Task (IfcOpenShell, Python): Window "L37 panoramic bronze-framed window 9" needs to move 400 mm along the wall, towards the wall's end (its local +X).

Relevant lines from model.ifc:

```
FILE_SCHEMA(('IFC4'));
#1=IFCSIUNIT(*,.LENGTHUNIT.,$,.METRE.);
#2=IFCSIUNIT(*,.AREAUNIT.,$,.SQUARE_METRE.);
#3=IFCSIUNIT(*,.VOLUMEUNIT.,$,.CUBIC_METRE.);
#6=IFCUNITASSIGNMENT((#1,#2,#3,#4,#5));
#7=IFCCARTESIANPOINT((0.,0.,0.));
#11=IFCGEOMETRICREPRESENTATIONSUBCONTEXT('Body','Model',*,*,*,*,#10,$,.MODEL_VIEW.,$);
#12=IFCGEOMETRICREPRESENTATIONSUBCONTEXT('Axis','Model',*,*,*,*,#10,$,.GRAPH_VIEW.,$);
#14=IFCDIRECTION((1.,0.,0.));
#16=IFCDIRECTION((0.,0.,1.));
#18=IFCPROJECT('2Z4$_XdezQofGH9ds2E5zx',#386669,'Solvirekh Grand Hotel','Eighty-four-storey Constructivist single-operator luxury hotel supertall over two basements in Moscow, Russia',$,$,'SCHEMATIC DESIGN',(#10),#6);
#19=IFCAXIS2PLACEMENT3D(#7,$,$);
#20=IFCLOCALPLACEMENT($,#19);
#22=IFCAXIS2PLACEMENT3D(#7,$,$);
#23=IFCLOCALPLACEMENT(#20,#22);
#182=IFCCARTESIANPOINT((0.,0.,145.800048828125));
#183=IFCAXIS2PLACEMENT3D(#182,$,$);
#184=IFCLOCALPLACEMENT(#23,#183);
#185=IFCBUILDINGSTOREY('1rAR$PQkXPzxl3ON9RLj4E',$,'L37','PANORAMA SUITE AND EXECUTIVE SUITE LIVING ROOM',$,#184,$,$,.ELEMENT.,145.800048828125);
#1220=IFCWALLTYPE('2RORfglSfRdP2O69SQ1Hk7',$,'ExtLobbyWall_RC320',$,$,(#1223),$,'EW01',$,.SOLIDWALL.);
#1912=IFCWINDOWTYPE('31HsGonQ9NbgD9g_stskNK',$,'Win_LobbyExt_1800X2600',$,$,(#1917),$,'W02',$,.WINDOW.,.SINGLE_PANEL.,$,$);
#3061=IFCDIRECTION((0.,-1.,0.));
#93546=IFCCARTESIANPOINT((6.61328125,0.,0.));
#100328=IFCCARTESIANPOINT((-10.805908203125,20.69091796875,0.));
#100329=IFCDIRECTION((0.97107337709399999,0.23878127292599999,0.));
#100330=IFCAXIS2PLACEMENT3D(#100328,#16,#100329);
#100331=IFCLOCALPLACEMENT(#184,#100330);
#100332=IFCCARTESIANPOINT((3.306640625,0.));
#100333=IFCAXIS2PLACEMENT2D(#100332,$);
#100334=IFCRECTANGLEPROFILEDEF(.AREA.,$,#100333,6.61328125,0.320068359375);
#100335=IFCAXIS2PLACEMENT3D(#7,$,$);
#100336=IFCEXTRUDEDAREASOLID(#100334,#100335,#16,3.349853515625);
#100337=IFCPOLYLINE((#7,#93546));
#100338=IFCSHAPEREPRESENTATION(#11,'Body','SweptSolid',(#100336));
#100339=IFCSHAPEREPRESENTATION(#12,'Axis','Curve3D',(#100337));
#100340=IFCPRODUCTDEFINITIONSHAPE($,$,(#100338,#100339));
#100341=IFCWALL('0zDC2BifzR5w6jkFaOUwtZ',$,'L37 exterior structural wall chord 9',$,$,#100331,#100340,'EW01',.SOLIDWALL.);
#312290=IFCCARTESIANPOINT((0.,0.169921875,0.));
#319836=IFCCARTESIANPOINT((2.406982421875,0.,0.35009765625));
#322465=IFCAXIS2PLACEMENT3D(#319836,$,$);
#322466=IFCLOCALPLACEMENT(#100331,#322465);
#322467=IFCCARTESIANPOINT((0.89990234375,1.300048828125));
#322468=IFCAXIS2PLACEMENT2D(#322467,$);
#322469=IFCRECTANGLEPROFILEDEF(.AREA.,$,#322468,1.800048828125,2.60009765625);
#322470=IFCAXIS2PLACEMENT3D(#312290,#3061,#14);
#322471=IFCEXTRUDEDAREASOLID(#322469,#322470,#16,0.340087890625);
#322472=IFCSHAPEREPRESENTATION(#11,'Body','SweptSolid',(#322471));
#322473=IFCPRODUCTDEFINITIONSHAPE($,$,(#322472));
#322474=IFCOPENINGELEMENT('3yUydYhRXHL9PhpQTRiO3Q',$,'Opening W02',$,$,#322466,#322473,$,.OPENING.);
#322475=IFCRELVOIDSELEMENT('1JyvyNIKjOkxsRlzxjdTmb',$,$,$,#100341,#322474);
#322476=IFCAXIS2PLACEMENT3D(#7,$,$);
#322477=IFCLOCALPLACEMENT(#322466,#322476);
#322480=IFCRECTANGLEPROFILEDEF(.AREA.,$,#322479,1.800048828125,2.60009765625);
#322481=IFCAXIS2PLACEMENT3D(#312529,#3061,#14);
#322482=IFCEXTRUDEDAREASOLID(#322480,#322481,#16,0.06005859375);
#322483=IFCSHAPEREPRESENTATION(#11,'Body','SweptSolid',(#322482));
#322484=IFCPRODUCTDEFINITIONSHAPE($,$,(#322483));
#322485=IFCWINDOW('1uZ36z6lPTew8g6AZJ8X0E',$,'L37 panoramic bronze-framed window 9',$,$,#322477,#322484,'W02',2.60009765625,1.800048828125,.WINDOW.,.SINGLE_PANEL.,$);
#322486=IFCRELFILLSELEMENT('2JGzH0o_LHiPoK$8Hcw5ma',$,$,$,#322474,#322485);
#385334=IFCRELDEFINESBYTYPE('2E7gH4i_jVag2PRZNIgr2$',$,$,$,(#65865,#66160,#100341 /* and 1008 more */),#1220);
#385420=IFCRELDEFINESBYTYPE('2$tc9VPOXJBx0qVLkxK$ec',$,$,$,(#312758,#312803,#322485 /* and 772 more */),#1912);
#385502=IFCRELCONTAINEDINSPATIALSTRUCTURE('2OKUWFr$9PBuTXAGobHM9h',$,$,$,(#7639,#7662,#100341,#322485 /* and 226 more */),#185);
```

```python
import ifcopenshell
import ifcopenshell.api.geometry
import ifcopenshell.util.placement
import ifcopenshell.util.unit

model = ifcopenshell.open("model.ifc")
unit_scale = ifcopenshell.util.unit.calculate_unit_scale(model)

window = model.by_id(322485)
opening = window.FillsVoids[0].RelatingOpeningElement
wall = opening.VoidsElements[0].RelatingBuildingElement

wall_matrix = ifcopenshell.util.placement.get_local_placement(wall.ObjectPlacement)
shift = wall_matrix[:3, 0] * 0.4 / unit_scale
before = ifcopenshell.util.placement.get_local_placement(window.ObjectPlacement)[:3, 3].copy()

# The window is placed relative to its opening, so it follows when the opening moves.
matrix = ifcopenshell.util.placement.get_local_placement(opening.ObjectPlacement)
matrix[:3, 3] += shift
ifcopenshell.api.geometry.edit_object_placement(
    model, product=opening, matrix=matrix, is_si=False, should_transform_children=True
)

after = ifcopenshell.util.placement.get_local_placement(window.ObjectPlacement)[:3, 3]
print("window moved by", (after - before).round(3) + 0.0)

model.write("model_v2.ifc")
```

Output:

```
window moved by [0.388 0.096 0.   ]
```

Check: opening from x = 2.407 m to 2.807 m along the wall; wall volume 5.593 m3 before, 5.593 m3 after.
